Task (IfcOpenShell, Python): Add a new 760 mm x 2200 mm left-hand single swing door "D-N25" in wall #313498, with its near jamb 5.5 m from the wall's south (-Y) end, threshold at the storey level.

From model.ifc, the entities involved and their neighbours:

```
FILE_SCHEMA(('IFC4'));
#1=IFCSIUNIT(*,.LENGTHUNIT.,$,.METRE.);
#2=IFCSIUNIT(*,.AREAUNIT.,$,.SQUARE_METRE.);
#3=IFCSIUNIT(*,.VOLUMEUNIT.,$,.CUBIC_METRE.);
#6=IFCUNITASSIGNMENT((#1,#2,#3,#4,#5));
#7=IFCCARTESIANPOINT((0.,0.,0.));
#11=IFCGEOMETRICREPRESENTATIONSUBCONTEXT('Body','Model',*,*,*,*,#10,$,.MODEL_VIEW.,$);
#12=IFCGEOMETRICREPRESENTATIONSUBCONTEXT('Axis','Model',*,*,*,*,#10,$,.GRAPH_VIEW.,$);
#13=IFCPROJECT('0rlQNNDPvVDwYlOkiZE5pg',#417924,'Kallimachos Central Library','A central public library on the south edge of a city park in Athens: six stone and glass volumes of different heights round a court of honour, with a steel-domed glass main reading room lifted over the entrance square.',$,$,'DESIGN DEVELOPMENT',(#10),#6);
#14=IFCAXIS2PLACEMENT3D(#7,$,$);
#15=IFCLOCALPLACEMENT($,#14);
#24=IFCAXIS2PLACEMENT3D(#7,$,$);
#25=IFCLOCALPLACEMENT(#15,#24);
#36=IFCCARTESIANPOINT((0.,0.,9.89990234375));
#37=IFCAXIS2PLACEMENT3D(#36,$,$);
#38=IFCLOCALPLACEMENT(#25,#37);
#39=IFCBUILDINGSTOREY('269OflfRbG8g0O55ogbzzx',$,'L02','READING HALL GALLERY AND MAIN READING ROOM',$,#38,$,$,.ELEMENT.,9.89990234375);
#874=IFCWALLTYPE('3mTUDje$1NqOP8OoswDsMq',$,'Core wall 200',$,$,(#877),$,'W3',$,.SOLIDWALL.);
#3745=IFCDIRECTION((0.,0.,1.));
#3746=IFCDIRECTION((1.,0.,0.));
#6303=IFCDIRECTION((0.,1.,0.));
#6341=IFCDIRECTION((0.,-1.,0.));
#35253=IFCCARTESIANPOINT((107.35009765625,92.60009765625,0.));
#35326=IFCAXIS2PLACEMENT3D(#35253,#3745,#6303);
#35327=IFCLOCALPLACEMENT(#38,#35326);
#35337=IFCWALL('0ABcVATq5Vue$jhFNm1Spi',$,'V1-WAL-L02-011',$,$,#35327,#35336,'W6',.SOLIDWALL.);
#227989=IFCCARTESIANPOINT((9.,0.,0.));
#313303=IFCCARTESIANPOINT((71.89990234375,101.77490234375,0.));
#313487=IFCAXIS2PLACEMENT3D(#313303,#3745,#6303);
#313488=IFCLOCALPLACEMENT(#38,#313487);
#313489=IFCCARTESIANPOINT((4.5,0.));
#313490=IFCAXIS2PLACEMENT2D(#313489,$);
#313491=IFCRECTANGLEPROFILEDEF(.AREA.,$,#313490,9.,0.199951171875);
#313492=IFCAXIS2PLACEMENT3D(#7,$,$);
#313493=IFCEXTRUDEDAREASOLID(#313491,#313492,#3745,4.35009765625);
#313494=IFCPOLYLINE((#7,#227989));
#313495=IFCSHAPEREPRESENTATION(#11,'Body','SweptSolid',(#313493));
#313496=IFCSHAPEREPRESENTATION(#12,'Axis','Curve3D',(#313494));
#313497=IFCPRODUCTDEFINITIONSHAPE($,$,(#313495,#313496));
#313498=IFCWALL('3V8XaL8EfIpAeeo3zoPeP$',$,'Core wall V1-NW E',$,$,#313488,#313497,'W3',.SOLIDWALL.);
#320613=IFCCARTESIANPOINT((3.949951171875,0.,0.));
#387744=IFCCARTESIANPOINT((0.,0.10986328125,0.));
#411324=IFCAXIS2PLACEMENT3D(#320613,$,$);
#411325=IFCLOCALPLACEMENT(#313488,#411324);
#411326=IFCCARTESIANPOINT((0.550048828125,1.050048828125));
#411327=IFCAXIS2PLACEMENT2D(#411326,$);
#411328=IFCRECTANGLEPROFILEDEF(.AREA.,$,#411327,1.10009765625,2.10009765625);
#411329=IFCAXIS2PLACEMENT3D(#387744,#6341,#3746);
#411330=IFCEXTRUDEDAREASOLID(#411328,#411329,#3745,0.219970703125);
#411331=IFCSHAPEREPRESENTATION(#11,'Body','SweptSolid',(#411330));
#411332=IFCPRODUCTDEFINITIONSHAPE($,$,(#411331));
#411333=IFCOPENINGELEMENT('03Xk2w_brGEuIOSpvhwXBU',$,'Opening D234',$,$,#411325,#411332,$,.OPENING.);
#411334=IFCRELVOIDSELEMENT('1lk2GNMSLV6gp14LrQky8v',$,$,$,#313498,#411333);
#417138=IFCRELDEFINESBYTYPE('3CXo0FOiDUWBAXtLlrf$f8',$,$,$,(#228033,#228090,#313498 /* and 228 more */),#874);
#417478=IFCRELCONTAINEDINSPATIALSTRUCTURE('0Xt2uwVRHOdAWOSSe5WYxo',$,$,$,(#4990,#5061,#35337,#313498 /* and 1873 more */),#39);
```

```python
import numpy as np
import ifcopenshell
import ifcopenshell.api.feature
import ifcopenshell.api.geometry
import ifcopenshell.api.root
import ifcopenshell.api.spatial
import ifcopenshell.geom
import ifcopenshell.util.element
import ifcopenshell.util.placement
import ifcopenshell.util.representation
import ifcopenshell.util.shape
import ifcopenshell.util.unit

model = ifcopenshell.open("model.ifc")
unit_scale = ifcopenshell.util.unit.calculate_unit_scale(model)
settings = ifcopenshell.geom.settings()


def volume(element):
    """Net volume in cubic metres, openings subtracted."""
    shape = ifcopenshell.geom.create_shape(settings, element)
    return ifcopenshell.util.shape.get_volume(shape.geometry)


wall = model.by_guid("3V8XaL8EfIpAeeo3zoPeP$")
storey = ifcopenshell.util.element.get_container(wall, ifc_class="IfcBuildingStorey")
context = ifcopenshell.util.representation.get_context(model, "Model", "Body", "MODEL_VIEW")
before = volume(wall)

width, height, from_end, sill = 0.76, 2.2, 5.5, 0.0  # metres

# The wall runs along its own X axis, and the end named is its -X end.
wall_shape = ifcopenshell.geom.create_shape(settings, wall)
x, y, z = ifcopenshell.util.shape.get_vertices(wall_shape.geometry).T
start = x.min() + from_end
face, thickness = float(y.min()), float(y.max() - y.min())
wall_matrix = ifcopenshell.util.placement.get_local_placement(wall.ObjectPlacement)
level = ifcopenshell.util.placement.get_local_placement(storey.ObjectPlacement)[2, 3]


def in_wall(x, y):
    """Placement at x, y metres in the wall's axes, at sill height."""
    matrix = wall_matrix.copy()
    matrix[:, 3] = wall_matrix @ np.array([x / unit_scale, y / unit_scale, 0.0, 1.0])
    matrix[2, 3] = level + sill / unit_scale
    return matrix


# Opening: a box that overshoots both wall faces by 50 mm.
opening = ifcopenshell.api.root.create_entity(model, ifc_class="IfcOpeningElement", predefined_type="OPENING")
box = ifcopenshell.api.geometry.add_wall_representation(
    model, context=context, length=width, height=height, thickness=thickness + 0.1
)
ifcopenshell.api.geometry.assign_representation(model, product=opening, representation=box)
ifcopenshell.api.geometry.edit_object_placement(model, product=opening, matrix=in_wall(start, face - 0.05), is_si=False)
ifcopenshell.api.feature.add_feature(model, feature=opening, element=wall)

door = ifcopenshell.api.root.create_entity(model, ifc_class="IfcDoor", name="D-N25", predefined_type="DOOR")
door.OverallWidth, door.OverallHeight = width / unit_scale, height / unit_scale
door.OperationType = "SINGLE_SWING_LEFT"
body = ifcopenshell.api.geometry.add_door_representation(
    model,
    context=context,
    overall_width=door.OverallWidth,
    overall_height=door.OverallHeight,
    operation_type="SINGLE_SWING_LEFT",
    lining_properties={"LiningDepth": thickness / unit_scale, "ThresholdDepth": thickness / unit_scale},
)
ifcopenshell.api.geometry.assign_representation(model, product=door, representation=body)
ifcopenshell.api.spatial.assign_container(model, products=[door], relating_structure=storey)
ifcopenshell.api.feature.add_filling(model, opening=opening, element=door)

# The lining spans the wall, so the door starts at the wall face.
ifcopenshell.api.geometry.edit_object_placement(model, product=door, matrix=in_wall(start, face), is_si=False)

after = volume(wall)

print(f"wall volume {before:.3f} -> {after:.3f} m3")

model.write("model-out.ifc")
```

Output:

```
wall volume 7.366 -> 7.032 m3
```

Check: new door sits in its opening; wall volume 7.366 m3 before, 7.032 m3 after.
